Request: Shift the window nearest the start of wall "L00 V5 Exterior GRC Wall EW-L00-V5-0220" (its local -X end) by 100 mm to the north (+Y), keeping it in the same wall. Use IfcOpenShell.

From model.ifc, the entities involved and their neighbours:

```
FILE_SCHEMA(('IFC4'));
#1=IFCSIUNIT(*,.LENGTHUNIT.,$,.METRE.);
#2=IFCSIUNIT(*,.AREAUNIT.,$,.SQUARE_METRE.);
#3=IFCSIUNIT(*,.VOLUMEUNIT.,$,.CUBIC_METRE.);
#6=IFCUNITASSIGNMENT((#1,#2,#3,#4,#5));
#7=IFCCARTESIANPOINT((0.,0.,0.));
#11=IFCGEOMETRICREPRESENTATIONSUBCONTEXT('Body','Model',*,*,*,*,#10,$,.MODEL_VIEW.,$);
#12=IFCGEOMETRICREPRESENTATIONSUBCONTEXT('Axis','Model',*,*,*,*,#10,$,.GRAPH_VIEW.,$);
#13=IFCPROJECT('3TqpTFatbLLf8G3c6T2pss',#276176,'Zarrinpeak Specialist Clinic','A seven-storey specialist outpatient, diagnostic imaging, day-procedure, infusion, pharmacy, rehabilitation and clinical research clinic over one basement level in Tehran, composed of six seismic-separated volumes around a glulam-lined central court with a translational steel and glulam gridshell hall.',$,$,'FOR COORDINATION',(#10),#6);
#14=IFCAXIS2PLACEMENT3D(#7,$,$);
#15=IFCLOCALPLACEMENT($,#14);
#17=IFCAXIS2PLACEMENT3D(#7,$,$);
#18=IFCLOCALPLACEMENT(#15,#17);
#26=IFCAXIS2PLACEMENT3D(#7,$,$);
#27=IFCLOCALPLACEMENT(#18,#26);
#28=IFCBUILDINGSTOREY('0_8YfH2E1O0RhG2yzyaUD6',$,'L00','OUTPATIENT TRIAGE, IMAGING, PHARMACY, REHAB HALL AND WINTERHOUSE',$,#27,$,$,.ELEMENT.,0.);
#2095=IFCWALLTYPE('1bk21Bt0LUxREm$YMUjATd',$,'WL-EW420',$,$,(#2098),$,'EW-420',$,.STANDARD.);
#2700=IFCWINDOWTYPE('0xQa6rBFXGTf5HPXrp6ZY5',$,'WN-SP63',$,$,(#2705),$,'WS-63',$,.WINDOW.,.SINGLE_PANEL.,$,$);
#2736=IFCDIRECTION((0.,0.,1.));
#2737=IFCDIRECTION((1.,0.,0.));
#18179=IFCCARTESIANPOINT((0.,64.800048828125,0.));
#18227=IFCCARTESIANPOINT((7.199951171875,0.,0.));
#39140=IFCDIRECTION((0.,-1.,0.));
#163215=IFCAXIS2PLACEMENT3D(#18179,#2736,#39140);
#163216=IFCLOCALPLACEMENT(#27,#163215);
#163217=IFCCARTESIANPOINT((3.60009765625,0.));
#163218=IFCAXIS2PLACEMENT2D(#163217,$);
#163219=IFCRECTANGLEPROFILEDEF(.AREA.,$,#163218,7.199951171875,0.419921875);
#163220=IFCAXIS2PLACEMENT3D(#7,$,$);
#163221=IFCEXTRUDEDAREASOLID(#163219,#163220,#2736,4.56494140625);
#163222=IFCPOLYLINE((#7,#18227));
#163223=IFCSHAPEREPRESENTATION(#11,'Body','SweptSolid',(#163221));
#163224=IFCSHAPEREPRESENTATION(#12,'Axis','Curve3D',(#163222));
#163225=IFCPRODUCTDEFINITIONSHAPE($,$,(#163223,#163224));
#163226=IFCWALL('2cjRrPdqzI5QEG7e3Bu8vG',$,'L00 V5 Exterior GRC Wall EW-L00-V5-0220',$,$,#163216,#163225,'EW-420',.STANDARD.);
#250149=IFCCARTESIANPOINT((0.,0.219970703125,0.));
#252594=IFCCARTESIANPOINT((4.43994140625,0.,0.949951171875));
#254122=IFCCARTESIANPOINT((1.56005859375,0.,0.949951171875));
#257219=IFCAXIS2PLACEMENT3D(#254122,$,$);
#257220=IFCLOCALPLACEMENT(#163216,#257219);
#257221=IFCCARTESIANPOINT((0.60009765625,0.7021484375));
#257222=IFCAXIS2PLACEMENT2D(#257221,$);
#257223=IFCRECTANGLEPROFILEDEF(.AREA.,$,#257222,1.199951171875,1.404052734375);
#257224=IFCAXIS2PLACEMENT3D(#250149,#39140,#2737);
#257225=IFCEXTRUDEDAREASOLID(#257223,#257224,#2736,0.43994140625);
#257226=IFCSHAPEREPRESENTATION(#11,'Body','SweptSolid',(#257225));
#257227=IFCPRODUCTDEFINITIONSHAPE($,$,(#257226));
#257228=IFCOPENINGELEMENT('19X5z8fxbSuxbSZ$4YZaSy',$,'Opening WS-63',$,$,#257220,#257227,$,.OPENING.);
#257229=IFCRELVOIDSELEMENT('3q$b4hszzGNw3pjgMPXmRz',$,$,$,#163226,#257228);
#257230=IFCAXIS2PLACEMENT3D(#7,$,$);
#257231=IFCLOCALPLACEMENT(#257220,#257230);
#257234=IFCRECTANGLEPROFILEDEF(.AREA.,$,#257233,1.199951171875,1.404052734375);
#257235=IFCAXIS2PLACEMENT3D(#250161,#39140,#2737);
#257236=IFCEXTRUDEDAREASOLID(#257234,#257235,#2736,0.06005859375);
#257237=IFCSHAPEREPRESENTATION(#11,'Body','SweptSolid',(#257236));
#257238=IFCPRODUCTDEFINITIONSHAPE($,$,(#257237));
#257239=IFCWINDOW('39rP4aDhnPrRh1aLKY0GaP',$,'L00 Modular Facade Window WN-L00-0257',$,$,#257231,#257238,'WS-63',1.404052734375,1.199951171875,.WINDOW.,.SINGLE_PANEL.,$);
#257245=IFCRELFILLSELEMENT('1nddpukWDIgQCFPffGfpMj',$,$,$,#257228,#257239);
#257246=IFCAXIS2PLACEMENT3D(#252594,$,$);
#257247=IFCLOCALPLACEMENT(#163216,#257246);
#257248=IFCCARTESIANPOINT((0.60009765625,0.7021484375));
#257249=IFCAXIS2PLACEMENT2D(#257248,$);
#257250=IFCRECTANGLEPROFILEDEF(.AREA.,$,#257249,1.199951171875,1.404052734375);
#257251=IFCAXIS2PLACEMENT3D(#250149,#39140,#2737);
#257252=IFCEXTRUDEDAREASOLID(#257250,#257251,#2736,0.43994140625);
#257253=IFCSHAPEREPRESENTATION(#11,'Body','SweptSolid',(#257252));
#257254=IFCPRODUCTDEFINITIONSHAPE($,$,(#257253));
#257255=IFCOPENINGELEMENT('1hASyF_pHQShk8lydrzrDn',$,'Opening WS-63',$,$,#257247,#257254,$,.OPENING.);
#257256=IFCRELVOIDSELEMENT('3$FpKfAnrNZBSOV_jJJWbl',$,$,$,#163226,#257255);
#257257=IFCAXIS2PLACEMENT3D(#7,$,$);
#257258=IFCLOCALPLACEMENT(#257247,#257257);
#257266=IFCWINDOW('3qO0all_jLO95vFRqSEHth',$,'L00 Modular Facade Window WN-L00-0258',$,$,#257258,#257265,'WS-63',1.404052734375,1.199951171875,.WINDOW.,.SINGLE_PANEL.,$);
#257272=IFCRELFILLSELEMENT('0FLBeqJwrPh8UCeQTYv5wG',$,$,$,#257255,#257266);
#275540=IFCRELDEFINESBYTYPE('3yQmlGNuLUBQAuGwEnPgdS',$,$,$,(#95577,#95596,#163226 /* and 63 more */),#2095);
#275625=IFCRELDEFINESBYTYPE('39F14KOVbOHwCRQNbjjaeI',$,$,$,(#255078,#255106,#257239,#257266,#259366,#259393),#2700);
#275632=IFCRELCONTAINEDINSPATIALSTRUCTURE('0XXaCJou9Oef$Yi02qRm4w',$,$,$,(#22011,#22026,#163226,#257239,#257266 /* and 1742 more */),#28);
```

```python
import ifcopenshell
import ifcopenshell.api.geometry
import ifcopenshell.util.placement
import ifcopenshell.util.unit

model = ifcopenshell.open("model.ifc")
unit_scale = ifcopenshell.util.unit.calculate_unit_scale(model)

window = model.by_guid("39rP4aDhnPrRh1aLKY0GaP")
opening = window.FillsVoids[0].RelatingOpeningElement
wall = opening.VoidsElements[0].RelatingBuildingElement

wall_matrix = ifcopenshell.util.placement.get_local_placement(wall.ObjectPlacement)
shift = wall_matrix[:3, 0] * -0.1 / unit_scale
before = ifcopenshell.util.placement.get_local_placement(window.ObjectPlacement)[:3, 3].copy()

# The window is placed relative to its opening, so it follows when the opening moves.
matrix = ifcopenshell.util.placement.get_local_placement(opening.ObjectPlacement)
matrix[:3, 3] += shift
ifcopenshell.api.geometry.edit_object_placement(
    model, product=opening, matrix=matrix, is_si=False, should_transform_children=True
)

after = ifcopenshell.util.placement.get_local_placement(window.ObjectPlacement)[:3, 3]
print("window moved by", (after - before).round(3) + 0.0)

model.write("model_rev.ifc")
```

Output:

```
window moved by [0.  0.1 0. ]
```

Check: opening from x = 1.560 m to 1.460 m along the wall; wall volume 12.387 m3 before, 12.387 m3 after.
